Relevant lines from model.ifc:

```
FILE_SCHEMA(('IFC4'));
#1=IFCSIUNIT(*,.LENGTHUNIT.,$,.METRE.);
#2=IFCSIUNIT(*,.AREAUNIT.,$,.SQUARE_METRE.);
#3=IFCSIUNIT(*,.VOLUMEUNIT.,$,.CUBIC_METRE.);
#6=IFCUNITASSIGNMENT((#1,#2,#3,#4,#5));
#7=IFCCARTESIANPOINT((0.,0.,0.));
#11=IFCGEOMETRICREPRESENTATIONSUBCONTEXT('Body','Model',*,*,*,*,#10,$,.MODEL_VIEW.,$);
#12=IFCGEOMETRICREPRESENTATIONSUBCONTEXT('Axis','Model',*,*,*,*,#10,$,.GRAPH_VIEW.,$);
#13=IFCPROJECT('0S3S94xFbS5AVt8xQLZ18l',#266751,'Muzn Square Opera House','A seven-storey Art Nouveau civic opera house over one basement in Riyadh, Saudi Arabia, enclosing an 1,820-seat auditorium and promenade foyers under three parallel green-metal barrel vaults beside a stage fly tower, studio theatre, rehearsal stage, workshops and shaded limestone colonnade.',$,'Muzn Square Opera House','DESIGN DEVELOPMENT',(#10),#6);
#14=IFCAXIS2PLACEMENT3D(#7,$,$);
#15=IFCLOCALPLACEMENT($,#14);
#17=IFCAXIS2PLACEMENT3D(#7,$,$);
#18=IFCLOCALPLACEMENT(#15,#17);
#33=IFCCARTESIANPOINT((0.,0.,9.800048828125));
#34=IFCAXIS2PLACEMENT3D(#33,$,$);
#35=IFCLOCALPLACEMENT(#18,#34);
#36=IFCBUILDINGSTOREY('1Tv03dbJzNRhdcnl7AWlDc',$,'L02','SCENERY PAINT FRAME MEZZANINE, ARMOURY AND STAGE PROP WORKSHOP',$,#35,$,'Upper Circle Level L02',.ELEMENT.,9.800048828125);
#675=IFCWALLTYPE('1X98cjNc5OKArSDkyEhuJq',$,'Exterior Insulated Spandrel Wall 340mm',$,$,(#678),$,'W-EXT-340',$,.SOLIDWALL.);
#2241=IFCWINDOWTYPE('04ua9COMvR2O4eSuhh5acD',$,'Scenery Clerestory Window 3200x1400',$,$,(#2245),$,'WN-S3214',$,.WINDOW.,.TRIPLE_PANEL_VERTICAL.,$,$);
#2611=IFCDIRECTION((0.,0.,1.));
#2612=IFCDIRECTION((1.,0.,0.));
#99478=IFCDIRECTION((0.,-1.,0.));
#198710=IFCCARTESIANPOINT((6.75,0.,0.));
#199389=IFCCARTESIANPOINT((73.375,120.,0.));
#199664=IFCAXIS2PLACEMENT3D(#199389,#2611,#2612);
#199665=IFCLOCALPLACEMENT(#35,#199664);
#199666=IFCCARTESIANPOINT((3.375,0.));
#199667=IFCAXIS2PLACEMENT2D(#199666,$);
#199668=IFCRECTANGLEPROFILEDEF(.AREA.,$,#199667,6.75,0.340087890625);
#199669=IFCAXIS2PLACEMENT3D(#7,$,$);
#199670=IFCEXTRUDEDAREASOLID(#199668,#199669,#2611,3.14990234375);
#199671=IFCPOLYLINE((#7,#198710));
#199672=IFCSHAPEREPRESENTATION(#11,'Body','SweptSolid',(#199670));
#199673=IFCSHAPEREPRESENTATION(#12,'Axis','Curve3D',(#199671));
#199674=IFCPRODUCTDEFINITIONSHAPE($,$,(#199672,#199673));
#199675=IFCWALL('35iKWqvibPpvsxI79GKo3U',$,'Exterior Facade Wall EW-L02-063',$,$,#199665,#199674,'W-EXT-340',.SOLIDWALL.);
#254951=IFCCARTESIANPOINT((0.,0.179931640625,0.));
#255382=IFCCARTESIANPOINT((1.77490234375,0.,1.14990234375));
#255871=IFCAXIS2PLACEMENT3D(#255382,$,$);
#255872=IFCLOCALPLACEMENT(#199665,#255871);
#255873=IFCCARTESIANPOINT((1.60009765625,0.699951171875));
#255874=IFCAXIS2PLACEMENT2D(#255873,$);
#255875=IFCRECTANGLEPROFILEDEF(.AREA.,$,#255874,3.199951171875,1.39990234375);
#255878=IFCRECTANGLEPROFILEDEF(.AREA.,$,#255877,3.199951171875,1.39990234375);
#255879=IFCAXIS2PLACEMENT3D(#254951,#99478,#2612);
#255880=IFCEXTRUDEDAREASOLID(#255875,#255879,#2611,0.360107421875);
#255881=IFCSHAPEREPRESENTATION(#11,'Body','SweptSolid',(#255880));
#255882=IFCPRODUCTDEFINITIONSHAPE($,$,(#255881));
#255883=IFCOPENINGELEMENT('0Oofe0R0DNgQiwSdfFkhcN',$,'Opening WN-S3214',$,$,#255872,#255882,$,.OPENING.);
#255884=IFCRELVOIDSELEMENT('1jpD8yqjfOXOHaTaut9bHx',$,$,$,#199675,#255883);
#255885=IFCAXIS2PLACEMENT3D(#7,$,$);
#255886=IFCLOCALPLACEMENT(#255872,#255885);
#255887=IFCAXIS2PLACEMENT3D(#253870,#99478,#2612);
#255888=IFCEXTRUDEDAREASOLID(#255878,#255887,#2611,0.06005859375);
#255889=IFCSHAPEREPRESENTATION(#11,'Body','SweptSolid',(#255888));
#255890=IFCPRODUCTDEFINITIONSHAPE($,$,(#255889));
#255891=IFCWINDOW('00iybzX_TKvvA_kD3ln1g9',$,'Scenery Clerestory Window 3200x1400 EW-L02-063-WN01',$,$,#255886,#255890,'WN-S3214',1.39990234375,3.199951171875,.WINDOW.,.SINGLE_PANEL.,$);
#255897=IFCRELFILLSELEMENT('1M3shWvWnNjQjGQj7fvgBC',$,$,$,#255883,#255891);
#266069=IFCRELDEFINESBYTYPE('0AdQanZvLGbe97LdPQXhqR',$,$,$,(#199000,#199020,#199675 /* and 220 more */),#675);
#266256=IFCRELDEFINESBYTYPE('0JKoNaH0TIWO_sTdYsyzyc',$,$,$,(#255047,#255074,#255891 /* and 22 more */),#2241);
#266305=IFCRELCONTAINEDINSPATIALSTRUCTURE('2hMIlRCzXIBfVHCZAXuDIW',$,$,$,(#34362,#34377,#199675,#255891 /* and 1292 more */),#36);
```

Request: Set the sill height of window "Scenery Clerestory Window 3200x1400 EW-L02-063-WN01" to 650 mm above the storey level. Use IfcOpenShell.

```python
import numpy as np
import ifcopenshell
import ifcopenshell.api.geometry
import ifcopenshell.geom
import ifcopenshell.util.element
import ifcopenshell.util.placement
import ifcopenshell.util.shape
import ifcopenshell.util.unit

model = ifcopenshell.open("model.ifc")
unit_scale = ifcopenshell.util.unit.calculate_unit_scale(model)

window = model.by_guid("00iybzX_TKvvA_kD3ln1g9")
opening = window.FillsVoids[0].RelatingOpeningElement
storey = ifcopenshell.util.element.get_container(window, ifc_class="IfcBuildingStorey")
level = ifcopenshell.util.placement.get_local_placement(storey.ObjectPlacement)[2, 3]

# The opening's origin need not be at the sill, so measure its lowest point.
shape = ifcopenshell.geom.create_shape(ifcopenshell.geom.settings(), opening)
bottom = ifcopenshell.util.shape.get_shape_bottom_elevation(shape, shape.geometry) / unit_scale
dz = level + 0.65 / unit_scale - bottom

shift = np.array([0.0, 0.0, dz])
# The window is placed relative to its opening, so it follows when the opening moves.
matrix = ifcopenshell.util.placement.get_local_placement(opening.ObjectPlacement)
matrix[:3, 3] += shift
ifcopenshell.api.geometry.edit_object_placement(
    model, product=opening, matrix=matrix, is_si=False, should_transform_children=True
)

print(f"moved by {dz * unit_scale:+.3f} m")

model.write("model_v2.ifc")
```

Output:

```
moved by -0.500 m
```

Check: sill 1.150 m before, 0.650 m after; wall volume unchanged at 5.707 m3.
